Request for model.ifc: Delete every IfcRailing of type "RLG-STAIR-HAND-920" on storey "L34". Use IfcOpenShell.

First a look at what the model holds.

```python
import ifcopenshell
import ifcopenshell.util.element

model = ifcopenshell.open("model.ifc")
print(model.schema)
storey = next(s for s in model.by_type("IfcBuildingStorey") if s.Name == "L34")
railings = [e for e in ifcopenshell.util.element.get_decomposition(storey) if e.is_a("IfcRailing")]
seen = {}
for e in railings:
    element_type = ifcopenshell.util.element.get_type(e)
    name = element_type.Name if element_type not in (None, e) else None
    seen[name] = seen.get(name, 0) + 1
for name, count in sorted(seen.items(), key=str):
    print(count, "x", name)
```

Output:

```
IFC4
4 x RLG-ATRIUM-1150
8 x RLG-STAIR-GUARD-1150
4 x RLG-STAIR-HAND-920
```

```python
import ifcopenshell
import ifcopenshell.api.root
import ifcopenshell.util.element

model = ifcopenshell.open("model.ifc")

storey = next(s for s in model.by_type("IfcBuildingStorey") if s.Name == "L34")
railings = [e for e in ifcopenshell.util.element.get_decomposition(storey) if e.is_a("IfcRailing")]
targets = [e for e in railings if (t := ifcopenshell.util.element.get_type(e)) not in (None, e) and t.Name == "RLG-STAIR-HAND-920"]

for e in targets:
    ifcopenshell.api.root.remove_product(model, product=e)
print(len(targets), "removed")

model.write("model_edited.ifc")
```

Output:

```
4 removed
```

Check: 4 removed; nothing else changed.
